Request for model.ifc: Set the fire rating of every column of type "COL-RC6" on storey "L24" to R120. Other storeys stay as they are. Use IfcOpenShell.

First a look at what the model holds.

```python
import ifcopenshell
import ifcopenshell.util.element

model = ifcopenshell.open("model.ifc")
print(model.schema)
storey = next(s for s in model.by_type("IfcBuildingStorey") if s.Name == "L24")
columns = [e for e in ifcopenshell.util.element.get_decomposition(storey) if e.is_a("IfcColumn")]
seen = {}
for e in columns:
    element_type = ifcopenshell.util.element.get_type(e)
    key = (element_type.Name if element_type != e and element_type else None, ifcopenshell.util.element.get_pset(e, "Pset_ColumnCommon", "FireRating"))
    seen[key] = seen.get(key, 0) + 1
for (name, value), count in sorted(seen.items(), key=str):
    print(count, "x", name, "|", value)
```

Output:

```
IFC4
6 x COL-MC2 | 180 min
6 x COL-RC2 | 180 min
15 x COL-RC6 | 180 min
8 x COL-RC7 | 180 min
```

```python
import ifcopenshell
import ifcopenshell.api.pset
import ifcopenshell.util.element

model = ifcopenshell.open("model.ifc")

storey = next(s for s in model.by_type("IfcBuildingStorey") if s.Name == "L24")
columns = [e for e in ifcopenshell.util.element.get_decomposition(storey) if e.is_a("IfcColumn")]

count = 0
for e in columns:
    element_type = ifcopenshell.util.element.get_type(e)
    if element_type in (None, e) or element_type.Name != "COL-RC6":
        continue
    found = ifcopenshell.util.element.get_pset(e, "Pset_ColumnCommon", should_inherit=False)
    if found:
        pset = model.by_id(found["id"])
        if len(ifcopenshell.util.element.get_elements_by_pset(pset)) > 1:
            pset = ifcopenshell.api.pset.unshare_pset(model, products=[e], pset=pset)[0]
    else:
        pset = ifcopenshell.api.pset.add_pset(model, product=e, name="Pset_ColumnCommon")
    ifcopenshell.api.pset.edit_pset(model, pset=pset, properties={"FireRating": "R120"})
    count += 1

print(count, "columns updated")

model.write("model_updated.ifc")
```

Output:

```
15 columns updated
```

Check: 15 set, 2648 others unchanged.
